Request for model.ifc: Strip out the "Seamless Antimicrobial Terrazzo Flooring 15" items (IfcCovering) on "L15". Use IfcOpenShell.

First a look at what the model holds.

```python
import ifcopenshell
import ifcopenshell.util.element

model = ifcopenshell.open("model.ifc")
print(model.schema)
storey = next(s for s in model.by_type("IfcBuildingStorey") if s.Name == "L15")
coverings = [e for e in ifcopenshell.util.element.get_decomposition(storey) if e.is_a("IfcCovering")]
seen = {}
for e in coverings:
    element_type = ifcopenshell.util.element.get_type(e)
    name = element_type.Name if element_type not in (None, e) else None
    seen[name] = seen.get(name, 0) + 1
for name, count in sorted(seen.items(), key=str):
    print(count, "x", name)
```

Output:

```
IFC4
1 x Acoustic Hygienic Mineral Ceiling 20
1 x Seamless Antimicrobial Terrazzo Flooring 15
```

```python
import ifcopenshell
import ifcopenshell.api.root
import ifcopenshell.util.element

model = ifcopenshell.open("model.ifc")

storey = next(s for s in model.by_type("IfcBuildingStorey") if s.Name == "L15")
coverings = [e for e in ifcopenshell.util.element.get_decomposition(storey) if e.is_a("IfcCovering")]
targets = [e for e in coverings if (t := ifcopenshell.util.element.get_type(e)) not in (None, e) and t.Name == "Seamless Antimicrobial Terrazzo Flooring 15"]

for e in targets:
    ifcopenshell.api.root.remove_product(model, product=e)
print(len(targets), "removed")

model.write("model_v2.ifc")
```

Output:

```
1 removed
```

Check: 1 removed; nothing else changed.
